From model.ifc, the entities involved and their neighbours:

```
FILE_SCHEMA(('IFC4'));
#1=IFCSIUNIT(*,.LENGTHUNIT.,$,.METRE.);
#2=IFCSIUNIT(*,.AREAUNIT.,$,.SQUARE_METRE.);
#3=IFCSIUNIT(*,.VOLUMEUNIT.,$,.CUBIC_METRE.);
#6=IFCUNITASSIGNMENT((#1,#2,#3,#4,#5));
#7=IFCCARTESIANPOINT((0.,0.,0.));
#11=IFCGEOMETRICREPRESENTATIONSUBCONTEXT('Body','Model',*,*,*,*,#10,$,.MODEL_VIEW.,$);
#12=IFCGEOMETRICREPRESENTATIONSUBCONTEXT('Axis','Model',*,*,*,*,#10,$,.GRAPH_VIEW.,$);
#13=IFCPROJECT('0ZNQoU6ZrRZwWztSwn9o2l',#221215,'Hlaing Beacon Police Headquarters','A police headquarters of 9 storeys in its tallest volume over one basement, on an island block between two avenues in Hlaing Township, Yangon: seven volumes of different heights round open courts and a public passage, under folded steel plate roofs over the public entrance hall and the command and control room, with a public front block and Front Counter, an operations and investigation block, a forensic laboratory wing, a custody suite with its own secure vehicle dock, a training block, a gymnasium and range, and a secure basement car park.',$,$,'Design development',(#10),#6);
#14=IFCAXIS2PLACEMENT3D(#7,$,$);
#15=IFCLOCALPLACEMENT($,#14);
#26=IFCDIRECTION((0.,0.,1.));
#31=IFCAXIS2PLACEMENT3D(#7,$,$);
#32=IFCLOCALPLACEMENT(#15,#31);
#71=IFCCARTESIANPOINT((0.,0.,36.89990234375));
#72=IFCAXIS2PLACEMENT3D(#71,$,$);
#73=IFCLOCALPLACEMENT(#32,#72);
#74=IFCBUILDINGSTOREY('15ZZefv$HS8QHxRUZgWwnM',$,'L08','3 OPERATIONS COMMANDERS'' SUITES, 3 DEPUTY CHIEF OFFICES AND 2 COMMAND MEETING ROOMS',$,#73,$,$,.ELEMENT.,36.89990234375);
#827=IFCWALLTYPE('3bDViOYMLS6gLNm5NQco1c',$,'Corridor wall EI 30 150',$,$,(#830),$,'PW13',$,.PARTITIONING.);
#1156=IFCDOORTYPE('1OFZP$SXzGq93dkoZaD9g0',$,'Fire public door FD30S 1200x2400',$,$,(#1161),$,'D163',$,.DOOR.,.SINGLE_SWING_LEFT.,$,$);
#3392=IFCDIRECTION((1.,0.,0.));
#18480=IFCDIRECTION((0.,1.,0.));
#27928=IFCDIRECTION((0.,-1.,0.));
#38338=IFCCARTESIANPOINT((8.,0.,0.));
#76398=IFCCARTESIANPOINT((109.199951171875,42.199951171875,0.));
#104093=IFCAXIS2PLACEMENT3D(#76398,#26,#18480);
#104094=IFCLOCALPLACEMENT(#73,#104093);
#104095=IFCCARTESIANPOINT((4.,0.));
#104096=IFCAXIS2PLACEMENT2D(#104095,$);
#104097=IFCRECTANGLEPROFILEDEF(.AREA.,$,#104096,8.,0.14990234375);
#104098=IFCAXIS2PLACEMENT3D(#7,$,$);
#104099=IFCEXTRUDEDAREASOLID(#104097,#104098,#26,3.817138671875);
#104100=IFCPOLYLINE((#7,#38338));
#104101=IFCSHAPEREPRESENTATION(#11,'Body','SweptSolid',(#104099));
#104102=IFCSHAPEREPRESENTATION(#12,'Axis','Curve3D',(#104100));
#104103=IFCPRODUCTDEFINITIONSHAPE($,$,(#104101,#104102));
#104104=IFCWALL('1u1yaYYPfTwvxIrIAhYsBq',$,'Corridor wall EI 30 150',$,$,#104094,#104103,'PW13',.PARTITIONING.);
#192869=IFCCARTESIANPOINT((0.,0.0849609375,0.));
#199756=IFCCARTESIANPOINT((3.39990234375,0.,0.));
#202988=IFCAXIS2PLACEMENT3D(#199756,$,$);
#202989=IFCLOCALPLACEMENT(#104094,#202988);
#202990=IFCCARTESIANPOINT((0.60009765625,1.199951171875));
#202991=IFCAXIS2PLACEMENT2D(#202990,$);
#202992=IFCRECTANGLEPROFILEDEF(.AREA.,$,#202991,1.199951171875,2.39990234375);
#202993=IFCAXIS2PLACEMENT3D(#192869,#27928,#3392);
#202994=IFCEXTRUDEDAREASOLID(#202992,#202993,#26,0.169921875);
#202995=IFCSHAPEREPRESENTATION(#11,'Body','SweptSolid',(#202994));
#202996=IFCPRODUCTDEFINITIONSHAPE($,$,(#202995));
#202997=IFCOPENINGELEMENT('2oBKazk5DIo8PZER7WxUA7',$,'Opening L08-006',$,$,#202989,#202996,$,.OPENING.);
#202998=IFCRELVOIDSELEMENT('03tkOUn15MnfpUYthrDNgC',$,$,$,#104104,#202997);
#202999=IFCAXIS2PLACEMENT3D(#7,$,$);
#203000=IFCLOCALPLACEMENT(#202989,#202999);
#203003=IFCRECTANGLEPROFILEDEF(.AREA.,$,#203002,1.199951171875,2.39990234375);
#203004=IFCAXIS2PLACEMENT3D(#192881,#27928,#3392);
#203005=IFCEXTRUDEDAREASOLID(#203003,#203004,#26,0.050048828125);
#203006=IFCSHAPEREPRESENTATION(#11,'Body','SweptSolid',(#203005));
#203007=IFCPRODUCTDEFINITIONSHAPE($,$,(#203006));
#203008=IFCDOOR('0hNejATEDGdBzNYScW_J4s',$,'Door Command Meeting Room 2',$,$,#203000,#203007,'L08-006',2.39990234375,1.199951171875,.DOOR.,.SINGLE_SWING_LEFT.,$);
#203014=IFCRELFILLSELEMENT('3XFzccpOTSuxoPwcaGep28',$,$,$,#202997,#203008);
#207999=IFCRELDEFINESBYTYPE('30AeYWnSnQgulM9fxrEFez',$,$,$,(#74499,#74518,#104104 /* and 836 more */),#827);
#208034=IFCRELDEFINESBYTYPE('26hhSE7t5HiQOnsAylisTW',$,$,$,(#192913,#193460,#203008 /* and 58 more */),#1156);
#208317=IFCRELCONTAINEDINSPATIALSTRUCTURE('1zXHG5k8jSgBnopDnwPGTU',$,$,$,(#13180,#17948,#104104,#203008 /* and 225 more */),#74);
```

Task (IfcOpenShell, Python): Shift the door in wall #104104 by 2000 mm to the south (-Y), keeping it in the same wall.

```python
import ifcopenshell
import ifcopenshell.api.geometry
import ifcopenshell.util.placement

model = ifcopenshell.open("model.ifc")

door = model.by_guid("0hNejATEDGdBzNYScW_J4s")
opening = door.FillsVoids[0].RelatingOpeningElement
wall = opening.VoidsElements[0].RelatingBuildingElement

wall_matrix = ifcopenshell.util.placement.get_local_placement(wall.ObjectPlacement)
shift = wall_matrix[:3, 0] * -2.0
before = ifcopenshell.util.placement.get_local_placement(door.ObjectPlacement)[:3, 3].copy()

# The door is placed relative to its opening, so it follows when the opening moves.
matrix = ifcopenshell.util.placement.get_local_placement(opening.ObjectPlacement)
matrix[:3, 3] += shift
ifcopenshell.api.geometry.edit_object_placement(
    model, product=opening, matrix=matrix, is_si=False, should_transform_children=True
)

after = ifcopenshell.util.placement.get_local_placement(door.ObjectPlacement)[:3, 3]
print("door moved by", (after - before).round(3) + 0.0)

model.write("model_v2.ifc")
```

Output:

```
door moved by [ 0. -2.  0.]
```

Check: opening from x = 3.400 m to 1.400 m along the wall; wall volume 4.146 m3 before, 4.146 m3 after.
